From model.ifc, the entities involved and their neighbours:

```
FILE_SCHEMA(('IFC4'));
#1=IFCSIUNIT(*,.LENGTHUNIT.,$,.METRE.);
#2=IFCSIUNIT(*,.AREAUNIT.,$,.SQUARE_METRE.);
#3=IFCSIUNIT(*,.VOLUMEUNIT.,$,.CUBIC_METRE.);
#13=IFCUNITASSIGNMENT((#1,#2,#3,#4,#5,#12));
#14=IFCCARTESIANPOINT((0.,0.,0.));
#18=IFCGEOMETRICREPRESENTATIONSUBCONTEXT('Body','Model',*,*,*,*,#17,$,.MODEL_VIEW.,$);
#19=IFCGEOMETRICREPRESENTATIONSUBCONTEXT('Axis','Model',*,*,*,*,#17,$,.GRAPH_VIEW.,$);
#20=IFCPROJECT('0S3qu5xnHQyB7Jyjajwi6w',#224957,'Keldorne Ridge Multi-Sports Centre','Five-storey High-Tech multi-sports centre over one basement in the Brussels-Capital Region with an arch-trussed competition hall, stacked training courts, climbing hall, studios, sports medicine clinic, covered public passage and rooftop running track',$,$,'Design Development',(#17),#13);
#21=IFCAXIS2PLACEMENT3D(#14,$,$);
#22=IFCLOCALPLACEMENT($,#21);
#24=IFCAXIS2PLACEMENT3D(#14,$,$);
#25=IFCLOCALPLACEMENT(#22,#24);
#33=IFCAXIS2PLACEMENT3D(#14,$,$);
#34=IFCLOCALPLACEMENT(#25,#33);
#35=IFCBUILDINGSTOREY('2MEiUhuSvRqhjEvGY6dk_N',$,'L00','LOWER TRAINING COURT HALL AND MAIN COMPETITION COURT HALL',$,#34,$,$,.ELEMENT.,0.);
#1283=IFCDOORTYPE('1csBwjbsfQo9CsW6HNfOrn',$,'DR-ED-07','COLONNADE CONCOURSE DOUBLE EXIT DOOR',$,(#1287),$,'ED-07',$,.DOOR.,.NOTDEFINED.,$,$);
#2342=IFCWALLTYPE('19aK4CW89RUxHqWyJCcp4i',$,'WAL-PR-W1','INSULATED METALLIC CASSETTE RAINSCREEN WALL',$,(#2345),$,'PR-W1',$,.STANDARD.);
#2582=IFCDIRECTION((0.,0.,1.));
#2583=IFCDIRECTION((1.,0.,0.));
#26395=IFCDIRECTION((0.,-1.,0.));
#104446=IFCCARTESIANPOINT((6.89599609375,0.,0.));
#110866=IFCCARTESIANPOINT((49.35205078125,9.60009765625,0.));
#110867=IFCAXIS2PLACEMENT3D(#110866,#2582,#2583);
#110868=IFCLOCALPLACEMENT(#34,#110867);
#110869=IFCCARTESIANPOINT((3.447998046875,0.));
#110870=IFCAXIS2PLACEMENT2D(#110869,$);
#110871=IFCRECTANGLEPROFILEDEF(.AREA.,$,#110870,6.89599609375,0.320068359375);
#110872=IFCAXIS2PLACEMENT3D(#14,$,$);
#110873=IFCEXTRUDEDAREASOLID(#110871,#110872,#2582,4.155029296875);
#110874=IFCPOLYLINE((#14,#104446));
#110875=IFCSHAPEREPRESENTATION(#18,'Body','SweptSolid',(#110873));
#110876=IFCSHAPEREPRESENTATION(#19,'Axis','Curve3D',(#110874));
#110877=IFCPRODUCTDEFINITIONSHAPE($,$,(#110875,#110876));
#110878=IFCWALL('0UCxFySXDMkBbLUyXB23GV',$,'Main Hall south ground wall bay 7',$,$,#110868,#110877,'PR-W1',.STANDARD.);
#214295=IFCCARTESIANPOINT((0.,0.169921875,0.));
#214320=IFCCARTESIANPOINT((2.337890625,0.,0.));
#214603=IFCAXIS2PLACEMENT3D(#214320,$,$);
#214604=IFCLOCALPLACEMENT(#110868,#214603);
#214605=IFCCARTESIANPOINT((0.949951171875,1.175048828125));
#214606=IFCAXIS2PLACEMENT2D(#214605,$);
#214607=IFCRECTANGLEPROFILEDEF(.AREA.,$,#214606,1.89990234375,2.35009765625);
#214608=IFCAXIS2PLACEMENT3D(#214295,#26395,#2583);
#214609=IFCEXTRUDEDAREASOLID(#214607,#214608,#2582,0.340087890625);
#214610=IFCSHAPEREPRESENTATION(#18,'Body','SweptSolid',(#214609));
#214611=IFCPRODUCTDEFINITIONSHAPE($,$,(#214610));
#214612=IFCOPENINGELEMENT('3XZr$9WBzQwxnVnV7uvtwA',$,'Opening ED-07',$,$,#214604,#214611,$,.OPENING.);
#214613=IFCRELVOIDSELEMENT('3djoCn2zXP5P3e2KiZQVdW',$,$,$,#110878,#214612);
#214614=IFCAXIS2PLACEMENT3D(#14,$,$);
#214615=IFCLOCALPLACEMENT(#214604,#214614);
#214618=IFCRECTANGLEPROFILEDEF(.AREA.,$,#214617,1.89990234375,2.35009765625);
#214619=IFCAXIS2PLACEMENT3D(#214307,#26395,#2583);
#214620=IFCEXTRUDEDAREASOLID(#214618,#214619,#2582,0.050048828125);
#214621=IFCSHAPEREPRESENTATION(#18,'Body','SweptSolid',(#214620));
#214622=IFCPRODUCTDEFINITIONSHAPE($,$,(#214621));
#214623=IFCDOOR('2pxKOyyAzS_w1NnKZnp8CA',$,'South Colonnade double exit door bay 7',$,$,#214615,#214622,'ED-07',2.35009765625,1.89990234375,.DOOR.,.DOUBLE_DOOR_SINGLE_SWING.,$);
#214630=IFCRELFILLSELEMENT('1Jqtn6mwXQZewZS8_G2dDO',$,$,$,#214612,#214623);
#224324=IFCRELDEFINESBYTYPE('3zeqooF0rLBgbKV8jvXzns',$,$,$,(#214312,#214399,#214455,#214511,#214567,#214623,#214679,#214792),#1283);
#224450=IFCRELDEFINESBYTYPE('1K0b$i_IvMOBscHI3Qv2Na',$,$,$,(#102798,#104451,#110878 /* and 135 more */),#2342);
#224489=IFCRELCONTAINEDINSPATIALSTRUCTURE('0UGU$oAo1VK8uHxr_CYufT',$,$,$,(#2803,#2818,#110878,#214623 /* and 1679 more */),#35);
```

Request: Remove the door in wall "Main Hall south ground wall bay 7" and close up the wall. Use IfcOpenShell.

```python
import ifcopenshell
import ifcopenshell.api.feature
import ifcopenshell.api.root
import ifcopenshell.geom
import ifcopenshell.util.shape

model = ifcopenshell.open("model.ifc")
settings = ifcopenshell.geom.settings()


def volume(element):
    """Net volume in cubic metres, openings subtracted."""
    shape = ifcopenshell.geom.create_shape(settings, element)
    return ifcopenshell.util.shape.get_volume(shape.geometry)


door = model.by_id(214623)
opening = door.FillsVoids[0].RelatingOpeningElement
wall = opening.VoidsElements[0].RelatingBuildingElement
before = volume(wall)

ifcopenshell.api.root.remove_product(model, product=door)
ifcopenshell.api.feature.remove_feature(model, feature=opening)

after = volume(wall)

print(f"wall volume {before:.3f} -> {after:.3f} m3")

model.write("model-out.ifc")
```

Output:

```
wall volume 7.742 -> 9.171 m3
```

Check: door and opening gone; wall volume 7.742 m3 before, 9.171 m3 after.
